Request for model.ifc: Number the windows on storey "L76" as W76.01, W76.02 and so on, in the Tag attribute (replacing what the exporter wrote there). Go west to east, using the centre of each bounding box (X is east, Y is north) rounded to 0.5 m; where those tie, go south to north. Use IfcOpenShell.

First a look at what the model holds.

```python
import ifcopenshell
import ifcopenshell.util.element
import ifcopenshell.util.placement

model = ifcopenshell.open("model.ifc")
print(model.schema)
storey = next(s for s in model.by_type("IfcBuildingStorey") if s.Name == "L76")
windows = [e for e in ifcopenshell.util.element.get_decomposition(storey) if e.is_a("IfcWindow")]
for e in sorted(windows, key=lambda e: e.id()):
    origin = ifcopenshell.util.placement.get_local_placement(e.ObjectPlacement)[:3, 3]
    print(e.id(), e.Tag, e.Name, origin.round(2) + 0.0, sep=" | ")
```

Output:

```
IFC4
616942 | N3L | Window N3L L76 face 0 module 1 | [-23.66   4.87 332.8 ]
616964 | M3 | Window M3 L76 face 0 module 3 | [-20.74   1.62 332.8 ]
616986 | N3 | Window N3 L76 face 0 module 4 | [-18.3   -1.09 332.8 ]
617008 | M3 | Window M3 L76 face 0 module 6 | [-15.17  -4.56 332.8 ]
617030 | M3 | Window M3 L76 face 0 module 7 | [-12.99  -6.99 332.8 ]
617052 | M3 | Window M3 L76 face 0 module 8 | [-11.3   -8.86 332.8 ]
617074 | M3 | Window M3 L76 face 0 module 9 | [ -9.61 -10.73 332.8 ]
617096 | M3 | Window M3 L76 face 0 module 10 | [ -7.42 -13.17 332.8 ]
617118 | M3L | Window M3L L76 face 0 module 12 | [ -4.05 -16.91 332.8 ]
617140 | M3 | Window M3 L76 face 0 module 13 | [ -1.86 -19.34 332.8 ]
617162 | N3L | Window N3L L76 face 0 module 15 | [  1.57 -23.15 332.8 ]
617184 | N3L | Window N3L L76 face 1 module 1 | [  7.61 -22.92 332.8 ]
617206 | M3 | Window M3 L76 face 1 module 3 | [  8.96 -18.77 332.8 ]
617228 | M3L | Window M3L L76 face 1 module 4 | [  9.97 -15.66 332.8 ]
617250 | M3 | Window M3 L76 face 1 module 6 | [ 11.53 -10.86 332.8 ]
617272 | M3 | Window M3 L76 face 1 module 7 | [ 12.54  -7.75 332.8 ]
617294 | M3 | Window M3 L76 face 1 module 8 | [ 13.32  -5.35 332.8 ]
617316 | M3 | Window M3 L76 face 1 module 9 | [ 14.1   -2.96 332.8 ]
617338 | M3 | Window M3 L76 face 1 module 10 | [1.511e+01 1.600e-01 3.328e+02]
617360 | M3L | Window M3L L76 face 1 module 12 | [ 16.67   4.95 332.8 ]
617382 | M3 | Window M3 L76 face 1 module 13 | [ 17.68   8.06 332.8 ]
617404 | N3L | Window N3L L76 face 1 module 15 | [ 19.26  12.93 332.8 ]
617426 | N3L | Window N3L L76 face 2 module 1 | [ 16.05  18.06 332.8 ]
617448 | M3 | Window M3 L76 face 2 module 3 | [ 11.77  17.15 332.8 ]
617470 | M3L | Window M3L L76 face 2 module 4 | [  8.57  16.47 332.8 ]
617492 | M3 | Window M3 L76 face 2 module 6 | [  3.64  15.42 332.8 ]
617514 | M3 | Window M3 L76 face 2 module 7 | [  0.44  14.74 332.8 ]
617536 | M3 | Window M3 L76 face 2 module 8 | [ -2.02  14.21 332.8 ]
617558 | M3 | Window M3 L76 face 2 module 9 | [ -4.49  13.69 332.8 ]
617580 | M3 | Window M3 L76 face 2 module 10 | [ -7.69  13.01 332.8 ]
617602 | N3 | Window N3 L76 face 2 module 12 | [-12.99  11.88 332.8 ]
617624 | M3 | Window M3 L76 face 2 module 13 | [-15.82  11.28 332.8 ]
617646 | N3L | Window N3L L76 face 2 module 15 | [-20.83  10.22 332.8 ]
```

```python
import ifcopenshell
import ifcopenshell.geom
import ifcopenshell.util.element
import ifcopenshell.util.shape

model = ifcopenshell.open("model.ifc")
settings = ifcopenshell.geom.settings()
settings.set("use-world-coords", True)


def centre(element):
    shape = ifcopenshell.geom.create_shape(settings, element)
    return ifcopenshell.util.shape.get_bbox_centroid(shape.geometry)


storey = next(s for s in model.by_type("IfcBuildingStorey") if s.Name == "L76")
windows = [e for e in ifcopenshell.util.element.get_decomposition(storey) if e.is_a("IfcWindow")]

# Insertion points can sit at a corner or the storey origin, so sort by the geometry (in metres).
centres = {e: centre(e) for e in windows}
windows.sort(key=lambda e: (round(centres[e][0] / 0.5), centres[e][1]))

for i, e in enumerate(windows, start=1):
    number = f"W76.{i:02d}"
    e.Tag = number
    print(e.id(), number)

model.write("model-out.ifc")
```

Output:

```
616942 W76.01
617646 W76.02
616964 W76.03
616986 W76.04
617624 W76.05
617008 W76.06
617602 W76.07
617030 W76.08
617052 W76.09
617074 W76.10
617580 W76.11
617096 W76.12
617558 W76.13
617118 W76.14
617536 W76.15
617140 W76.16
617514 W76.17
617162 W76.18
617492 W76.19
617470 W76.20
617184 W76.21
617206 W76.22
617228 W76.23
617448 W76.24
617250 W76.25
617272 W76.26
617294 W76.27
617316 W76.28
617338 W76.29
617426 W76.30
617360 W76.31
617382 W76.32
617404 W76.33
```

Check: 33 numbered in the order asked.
